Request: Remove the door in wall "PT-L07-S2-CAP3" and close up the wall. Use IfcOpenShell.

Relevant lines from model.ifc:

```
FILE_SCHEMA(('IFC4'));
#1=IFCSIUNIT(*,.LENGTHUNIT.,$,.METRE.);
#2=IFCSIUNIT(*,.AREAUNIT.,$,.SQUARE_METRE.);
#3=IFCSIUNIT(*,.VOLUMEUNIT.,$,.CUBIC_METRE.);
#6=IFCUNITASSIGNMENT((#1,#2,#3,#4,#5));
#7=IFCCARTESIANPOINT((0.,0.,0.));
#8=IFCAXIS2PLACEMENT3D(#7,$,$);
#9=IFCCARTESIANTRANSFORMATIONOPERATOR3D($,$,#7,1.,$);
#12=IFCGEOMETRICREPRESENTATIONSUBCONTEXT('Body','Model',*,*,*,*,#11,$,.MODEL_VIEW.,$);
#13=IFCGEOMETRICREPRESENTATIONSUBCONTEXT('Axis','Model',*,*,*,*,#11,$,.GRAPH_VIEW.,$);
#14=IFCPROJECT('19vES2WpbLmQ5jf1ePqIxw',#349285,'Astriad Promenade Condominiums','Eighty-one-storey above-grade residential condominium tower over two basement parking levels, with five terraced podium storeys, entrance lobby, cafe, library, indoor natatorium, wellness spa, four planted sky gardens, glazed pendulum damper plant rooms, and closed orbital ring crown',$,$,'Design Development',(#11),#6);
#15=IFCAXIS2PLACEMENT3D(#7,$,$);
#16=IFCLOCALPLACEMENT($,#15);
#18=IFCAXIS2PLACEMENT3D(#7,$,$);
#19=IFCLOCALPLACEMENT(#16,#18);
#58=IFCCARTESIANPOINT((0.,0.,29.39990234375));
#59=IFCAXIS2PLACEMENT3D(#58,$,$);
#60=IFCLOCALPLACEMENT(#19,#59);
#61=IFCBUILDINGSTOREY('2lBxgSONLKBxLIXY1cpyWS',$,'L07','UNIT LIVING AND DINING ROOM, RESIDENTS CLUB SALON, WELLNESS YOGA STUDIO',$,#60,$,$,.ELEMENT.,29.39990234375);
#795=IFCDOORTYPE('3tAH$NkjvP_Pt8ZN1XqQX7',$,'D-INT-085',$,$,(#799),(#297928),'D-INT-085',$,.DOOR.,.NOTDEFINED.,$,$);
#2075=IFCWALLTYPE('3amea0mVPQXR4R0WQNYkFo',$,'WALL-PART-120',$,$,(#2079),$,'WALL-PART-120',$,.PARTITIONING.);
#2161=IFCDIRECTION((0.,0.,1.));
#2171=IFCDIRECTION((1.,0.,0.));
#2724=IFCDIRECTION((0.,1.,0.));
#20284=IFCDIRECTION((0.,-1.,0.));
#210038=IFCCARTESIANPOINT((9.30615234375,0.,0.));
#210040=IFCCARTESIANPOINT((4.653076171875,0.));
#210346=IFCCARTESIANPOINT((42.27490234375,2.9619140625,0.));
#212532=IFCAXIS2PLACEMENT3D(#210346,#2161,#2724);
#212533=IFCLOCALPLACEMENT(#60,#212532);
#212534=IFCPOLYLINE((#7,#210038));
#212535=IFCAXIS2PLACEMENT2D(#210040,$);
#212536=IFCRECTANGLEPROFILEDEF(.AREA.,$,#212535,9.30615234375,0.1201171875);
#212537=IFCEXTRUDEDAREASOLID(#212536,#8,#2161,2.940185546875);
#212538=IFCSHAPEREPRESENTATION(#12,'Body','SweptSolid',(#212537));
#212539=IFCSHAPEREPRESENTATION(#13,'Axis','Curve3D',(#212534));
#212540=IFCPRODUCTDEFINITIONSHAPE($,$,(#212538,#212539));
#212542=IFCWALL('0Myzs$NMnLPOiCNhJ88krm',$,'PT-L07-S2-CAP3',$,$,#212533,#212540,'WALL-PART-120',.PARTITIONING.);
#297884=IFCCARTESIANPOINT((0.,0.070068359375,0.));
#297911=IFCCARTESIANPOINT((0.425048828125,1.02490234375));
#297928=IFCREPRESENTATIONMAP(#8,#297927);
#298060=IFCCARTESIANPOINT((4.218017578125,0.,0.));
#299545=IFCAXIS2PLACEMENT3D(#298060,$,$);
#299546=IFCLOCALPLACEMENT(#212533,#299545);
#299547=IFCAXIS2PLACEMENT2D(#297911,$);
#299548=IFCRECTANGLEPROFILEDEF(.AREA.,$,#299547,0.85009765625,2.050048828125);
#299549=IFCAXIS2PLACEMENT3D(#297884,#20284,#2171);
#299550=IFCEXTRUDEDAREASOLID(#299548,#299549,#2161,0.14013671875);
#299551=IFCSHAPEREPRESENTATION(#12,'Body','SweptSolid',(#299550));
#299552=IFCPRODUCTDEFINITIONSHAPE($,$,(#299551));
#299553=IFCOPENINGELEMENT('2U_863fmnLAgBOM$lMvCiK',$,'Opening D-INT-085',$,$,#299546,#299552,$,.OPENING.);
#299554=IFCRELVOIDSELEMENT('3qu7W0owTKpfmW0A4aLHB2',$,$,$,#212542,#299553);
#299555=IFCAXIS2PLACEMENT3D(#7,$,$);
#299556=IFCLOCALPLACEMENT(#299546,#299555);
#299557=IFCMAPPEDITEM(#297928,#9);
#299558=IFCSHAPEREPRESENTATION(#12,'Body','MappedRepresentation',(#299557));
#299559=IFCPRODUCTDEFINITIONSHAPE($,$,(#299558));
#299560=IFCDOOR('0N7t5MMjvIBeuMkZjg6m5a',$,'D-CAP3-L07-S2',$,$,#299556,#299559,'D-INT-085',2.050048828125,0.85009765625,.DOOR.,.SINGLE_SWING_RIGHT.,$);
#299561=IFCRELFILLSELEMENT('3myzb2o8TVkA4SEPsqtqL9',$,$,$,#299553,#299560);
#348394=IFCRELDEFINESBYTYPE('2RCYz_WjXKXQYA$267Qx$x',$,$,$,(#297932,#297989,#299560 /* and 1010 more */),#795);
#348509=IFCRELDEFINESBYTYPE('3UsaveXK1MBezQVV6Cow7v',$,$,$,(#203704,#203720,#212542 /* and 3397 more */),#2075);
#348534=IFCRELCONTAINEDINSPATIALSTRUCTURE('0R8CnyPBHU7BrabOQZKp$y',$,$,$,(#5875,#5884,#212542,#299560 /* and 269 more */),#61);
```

```python
import ifcopenshell
import ifcopenshell.api.feature
import ifcopenshell.api.root
import ifcopenshell.geom
import ifcopenshell.util.shape

model = ifcopenshell.open("model.ifc")
settings = ifcopenshell.geom.settings()


def volume(element):
    """Net volume in cubic metres, openings subtracted."""
    shape = ifcopenshell.geom.create_shape(settings, element)
    return ifcopenshell.util.shape.get_volume(shape.geometry)


door = model.by_guid("0N7t5MMjvIBeuMkZjg6m5a")
opening = door.FillsVoids[0].RelatingOpeningElement
wall = opening.VoidsElements[0].RelatingBuildingElement
before = volume(wall)

ifcopenshell.api.root.remove_product(model, product=door)
ifcopenshell.api.feature.remove_feature(model, feature=opening)

after = volume(wall)

print(f"wall volume {before:.3f} -> {after:.3f} m3")

model.write("model_rev.ifc")
```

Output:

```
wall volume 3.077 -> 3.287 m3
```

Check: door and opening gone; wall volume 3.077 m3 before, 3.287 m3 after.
